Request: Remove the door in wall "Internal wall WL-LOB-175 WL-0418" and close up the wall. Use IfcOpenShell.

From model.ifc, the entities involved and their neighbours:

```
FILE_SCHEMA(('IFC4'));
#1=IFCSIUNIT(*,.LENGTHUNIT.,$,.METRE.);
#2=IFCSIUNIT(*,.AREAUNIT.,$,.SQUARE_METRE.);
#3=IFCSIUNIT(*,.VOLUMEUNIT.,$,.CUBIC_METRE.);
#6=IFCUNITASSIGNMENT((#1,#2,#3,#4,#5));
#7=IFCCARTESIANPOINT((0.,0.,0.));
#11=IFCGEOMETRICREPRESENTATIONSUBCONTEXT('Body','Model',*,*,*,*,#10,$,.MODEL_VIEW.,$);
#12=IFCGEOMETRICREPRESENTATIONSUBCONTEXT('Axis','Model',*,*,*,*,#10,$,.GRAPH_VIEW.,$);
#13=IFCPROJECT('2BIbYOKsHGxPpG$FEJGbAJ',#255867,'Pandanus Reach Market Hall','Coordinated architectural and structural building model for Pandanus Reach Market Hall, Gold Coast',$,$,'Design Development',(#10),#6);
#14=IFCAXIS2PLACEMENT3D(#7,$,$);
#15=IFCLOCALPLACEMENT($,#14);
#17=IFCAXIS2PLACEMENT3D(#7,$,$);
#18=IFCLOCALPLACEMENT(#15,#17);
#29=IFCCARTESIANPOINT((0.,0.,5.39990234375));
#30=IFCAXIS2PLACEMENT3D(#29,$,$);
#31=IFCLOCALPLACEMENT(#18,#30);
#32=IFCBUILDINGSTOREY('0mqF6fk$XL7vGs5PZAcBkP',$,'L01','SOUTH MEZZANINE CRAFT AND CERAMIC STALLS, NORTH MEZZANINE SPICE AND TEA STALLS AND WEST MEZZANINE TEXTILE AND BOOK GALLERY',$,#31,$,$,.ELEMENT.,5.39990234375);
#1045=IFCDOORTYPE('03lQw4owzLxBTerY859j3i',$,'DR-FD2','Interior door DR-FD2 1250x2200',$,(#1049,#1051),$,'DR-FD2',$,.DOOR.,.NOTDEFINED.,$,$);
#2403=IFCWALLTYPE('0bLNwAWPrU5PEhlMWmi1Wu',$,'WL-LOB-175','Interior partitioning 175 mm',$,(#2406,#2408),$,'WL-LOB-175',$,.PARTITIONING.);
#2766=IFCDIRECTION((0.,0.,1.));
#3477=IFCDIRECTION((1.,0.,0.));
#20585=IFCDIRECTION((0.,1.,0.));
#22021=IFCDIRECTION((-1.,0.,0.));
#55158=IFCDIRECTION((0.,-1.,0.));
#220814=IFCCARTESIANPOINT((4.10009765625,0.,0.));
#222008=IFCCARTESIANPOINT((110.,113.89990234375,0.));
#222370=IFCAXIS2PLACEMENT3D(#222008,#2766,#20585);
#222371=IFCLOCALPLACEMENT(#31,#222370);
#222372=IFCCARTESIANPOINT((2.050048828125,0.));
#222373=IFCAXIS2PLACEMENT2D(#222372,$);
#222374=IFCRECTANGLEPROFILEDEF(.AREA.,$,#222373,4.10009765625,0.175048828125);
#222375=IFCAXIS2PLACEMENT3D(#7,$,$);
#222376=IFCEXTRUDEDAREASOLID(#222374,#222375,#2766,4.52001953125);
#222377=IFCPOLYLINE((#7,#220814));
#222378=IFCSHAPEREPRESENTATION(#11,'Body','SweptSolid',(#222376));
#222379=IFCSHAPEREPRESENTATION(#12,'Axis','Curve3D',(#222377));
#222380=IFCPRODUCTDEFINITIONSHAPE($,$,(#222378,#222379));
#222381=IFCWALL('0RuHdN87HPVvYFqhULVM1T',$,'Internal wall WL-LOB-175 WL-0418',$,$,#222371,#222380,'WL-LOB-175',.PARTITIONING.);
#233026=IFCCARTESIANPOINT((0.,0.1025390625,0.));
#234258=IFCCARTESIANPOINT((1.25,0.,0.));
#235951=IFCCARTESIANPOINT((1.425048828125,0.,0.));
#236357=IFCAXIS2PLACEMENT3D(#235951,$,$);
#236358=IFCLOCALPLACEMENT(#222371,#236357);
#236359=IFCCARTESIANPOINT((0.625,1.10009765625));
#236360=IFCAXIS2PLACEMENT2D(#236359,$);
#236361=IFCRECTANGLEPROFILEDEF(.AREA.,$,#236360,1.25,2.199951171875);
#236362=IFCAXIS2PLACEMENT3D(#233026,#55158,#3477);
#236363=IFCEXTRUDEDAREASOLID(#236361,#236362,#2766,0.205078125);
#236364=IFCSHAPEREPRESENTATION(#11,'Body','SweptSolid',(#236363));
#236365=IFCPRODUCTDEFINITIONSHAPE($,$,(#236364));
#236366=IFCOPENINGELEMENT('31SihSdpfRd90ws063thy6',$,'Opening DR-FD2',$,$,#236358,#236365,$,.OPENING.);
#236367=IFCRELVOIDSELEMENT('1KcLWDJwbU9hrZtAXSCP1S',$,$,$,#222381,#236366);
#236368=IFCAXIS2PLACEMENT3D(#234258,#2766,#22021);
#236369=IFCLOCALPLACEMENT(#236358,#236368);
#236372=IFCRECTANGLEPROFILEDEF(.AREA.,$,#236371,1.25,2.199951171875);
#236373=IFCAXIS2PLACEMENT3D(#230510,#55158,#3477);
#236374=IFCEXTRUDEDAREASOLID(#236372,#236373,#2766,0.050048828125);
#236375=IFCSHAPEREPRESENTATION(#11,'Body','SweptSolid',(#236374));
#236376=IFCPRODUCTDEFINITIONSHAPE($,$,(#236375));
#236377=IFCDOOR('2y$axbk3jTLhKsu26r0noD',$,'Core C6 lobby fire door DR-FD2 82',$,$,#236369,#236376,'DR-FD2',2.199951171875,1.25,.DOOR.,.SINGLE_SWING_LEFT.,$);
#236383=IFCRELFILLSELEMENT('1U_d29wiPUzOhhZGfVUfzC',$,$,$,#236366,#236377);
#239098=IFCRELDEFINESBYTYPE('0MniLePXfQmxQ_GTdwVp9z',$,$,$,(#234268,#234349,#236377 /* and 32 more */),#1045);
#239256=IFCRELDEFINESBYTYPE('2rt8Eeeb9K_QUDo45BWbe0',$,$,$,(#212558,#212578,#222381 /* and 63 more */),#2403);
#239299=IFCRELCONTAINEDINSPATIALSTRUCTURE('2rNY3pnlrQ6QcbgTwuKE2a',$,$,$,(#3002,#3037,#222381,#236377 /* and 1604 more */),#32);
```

```python
import ifcopenshell
import ifcopenshell.api.feature
import ifcopenshell.api.root
import ifcopenshell.geom
import ifcopenshell.util.shape

model = ifcopenshell.open("model.ifc")
settings = ifcopenshell.geom.settings()


def volume(element):
    """Net volume in cubic metres, openings subtracted."""
    shape = ifcopenshell.geom.create_shape(settings, element)
    return ifcopenshell.util.shape.get_volume(shape.geometry)


door = model.by_guid("2y$axbk3jTLhKsu26r0noD")
opening = door.FillsVoids[0].RelatingOpeningElement
wall = opening.VoidsElements[0].RelatingBuildingElement
before = volume(wall)

ifcopenshell.api.root.remove_product(model, product=door)
ifcopenshell.api.feature.remove_feature(model, feature=opening)

after = volume(wall)

print(f"wall volume {before:.3f} -> {after:.3f} m3")

model.write("model_edited.ifc")
```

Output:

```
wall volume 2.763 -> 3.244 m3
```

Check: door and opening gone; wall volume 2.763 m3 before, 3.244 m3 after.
